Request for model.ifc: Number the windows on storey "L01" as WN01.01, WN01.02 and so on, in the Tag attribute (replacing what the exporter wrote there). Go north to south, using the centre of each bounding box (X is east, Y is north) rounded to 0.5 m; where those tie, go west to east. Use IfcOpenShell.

First a look at what the model holds.

```python
import ifcopenshell
import ifcopenshell.util.element
import ifcopenshell.util.placement

model = ifcopenshell.open("model.ifc")
print(model.schema)
storey = next(s for s in model.by_type("IfcBuildingStorey") if s.Name == "L01")
windows = [e for e in ifcopenshell.util.element.get_decomposition(storey) if e.is_a("IfcWindow")]
for e in sorted(windows, key=lambda e: e.id()):
    origin = ifcopenshell.util.placement.get_local_placement(e.ObjectPlacement)[:3, 3]
    print(e.id(), e.Tag, e.Name, origin.round(2) + 0.0, sep=" | ")
```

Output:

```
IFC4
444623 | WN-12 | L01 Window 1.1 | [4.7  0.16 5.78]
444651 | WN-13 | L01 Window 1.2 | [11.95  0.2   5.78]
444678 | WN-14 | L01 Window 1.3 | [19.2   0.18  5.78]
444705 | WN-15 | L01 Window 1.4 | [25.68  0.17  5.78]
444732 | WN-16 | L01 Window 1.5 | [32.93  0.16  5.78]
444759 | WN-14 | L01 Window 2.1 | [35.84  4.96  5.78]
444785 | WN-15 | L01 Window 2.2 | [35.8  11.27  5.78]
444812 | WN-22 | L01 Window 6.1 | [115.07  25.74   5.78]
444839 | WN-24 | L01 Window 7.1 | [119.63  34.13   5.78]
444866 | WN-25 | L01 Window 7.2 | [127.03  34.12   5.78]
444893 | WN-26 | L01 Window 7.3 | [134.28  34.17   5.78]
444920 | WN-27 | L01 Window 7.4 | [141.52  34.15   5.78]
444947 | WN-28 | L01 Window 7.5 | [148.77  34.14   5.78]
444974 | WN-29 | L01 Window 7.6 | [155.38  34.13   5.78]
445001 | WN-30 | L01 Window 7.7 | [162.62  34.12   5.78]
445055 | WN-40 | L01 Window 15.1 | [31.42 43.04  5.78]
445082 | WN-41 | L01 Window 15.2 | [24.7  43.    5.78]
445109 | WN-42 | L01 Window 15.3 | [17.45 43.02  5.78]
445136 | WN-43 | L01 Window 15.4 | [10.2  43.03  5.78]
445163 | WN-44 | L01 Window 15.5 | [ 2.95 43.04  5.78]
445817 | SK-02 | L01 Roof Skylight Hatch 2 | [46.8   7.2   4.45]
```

```python
import ifcopenshell
import ifcopenshell.geom
import ifcopenshell.util.element
import ifcopenshell.util.shape

model = ifcopenshell.open("model.ifc")
settings = ifcopenshell.geom.settings()
settings.set("use-world-coords", True)


def centre(element):
    shape = ifcopenshell.geom.create_shape(settings, element)
    return ifcopenshell.util.shape.get_bbox_centroid(shape.geometry)


storey = next(s for s in model.by_type("IfcBuildingStorey") if s.Name == "L01")
windows = [e for e in ifcopenshell.util.element.get_decomposition(storey) if e.is_a("IfcWindow")]

# Insertion points can sit at a corner or the storey origin, so sort by the geometry (in metres).
centres = {e: centre(e) for e in windows}
windows.sort(key=lambda e: (-round(centres[e][1] / 0.5), centres[e][0]))

for i, e in enumerate(windows, start=1):
    number = f"WN01.{i:02d}"
    e.Tag = number
    print(e.id(), number)

model.write("model_updated.ifc")
```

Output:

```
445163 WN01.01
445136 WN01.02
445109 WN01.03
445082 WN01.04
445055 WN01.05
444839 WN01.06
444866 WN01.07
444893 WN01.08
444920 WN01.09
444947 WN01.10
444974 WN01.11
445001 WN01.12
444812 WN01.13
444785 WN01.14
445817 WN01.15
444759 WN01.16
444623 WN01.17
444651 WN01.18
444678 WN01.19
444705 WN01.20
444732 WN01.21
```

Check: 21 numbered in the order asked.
